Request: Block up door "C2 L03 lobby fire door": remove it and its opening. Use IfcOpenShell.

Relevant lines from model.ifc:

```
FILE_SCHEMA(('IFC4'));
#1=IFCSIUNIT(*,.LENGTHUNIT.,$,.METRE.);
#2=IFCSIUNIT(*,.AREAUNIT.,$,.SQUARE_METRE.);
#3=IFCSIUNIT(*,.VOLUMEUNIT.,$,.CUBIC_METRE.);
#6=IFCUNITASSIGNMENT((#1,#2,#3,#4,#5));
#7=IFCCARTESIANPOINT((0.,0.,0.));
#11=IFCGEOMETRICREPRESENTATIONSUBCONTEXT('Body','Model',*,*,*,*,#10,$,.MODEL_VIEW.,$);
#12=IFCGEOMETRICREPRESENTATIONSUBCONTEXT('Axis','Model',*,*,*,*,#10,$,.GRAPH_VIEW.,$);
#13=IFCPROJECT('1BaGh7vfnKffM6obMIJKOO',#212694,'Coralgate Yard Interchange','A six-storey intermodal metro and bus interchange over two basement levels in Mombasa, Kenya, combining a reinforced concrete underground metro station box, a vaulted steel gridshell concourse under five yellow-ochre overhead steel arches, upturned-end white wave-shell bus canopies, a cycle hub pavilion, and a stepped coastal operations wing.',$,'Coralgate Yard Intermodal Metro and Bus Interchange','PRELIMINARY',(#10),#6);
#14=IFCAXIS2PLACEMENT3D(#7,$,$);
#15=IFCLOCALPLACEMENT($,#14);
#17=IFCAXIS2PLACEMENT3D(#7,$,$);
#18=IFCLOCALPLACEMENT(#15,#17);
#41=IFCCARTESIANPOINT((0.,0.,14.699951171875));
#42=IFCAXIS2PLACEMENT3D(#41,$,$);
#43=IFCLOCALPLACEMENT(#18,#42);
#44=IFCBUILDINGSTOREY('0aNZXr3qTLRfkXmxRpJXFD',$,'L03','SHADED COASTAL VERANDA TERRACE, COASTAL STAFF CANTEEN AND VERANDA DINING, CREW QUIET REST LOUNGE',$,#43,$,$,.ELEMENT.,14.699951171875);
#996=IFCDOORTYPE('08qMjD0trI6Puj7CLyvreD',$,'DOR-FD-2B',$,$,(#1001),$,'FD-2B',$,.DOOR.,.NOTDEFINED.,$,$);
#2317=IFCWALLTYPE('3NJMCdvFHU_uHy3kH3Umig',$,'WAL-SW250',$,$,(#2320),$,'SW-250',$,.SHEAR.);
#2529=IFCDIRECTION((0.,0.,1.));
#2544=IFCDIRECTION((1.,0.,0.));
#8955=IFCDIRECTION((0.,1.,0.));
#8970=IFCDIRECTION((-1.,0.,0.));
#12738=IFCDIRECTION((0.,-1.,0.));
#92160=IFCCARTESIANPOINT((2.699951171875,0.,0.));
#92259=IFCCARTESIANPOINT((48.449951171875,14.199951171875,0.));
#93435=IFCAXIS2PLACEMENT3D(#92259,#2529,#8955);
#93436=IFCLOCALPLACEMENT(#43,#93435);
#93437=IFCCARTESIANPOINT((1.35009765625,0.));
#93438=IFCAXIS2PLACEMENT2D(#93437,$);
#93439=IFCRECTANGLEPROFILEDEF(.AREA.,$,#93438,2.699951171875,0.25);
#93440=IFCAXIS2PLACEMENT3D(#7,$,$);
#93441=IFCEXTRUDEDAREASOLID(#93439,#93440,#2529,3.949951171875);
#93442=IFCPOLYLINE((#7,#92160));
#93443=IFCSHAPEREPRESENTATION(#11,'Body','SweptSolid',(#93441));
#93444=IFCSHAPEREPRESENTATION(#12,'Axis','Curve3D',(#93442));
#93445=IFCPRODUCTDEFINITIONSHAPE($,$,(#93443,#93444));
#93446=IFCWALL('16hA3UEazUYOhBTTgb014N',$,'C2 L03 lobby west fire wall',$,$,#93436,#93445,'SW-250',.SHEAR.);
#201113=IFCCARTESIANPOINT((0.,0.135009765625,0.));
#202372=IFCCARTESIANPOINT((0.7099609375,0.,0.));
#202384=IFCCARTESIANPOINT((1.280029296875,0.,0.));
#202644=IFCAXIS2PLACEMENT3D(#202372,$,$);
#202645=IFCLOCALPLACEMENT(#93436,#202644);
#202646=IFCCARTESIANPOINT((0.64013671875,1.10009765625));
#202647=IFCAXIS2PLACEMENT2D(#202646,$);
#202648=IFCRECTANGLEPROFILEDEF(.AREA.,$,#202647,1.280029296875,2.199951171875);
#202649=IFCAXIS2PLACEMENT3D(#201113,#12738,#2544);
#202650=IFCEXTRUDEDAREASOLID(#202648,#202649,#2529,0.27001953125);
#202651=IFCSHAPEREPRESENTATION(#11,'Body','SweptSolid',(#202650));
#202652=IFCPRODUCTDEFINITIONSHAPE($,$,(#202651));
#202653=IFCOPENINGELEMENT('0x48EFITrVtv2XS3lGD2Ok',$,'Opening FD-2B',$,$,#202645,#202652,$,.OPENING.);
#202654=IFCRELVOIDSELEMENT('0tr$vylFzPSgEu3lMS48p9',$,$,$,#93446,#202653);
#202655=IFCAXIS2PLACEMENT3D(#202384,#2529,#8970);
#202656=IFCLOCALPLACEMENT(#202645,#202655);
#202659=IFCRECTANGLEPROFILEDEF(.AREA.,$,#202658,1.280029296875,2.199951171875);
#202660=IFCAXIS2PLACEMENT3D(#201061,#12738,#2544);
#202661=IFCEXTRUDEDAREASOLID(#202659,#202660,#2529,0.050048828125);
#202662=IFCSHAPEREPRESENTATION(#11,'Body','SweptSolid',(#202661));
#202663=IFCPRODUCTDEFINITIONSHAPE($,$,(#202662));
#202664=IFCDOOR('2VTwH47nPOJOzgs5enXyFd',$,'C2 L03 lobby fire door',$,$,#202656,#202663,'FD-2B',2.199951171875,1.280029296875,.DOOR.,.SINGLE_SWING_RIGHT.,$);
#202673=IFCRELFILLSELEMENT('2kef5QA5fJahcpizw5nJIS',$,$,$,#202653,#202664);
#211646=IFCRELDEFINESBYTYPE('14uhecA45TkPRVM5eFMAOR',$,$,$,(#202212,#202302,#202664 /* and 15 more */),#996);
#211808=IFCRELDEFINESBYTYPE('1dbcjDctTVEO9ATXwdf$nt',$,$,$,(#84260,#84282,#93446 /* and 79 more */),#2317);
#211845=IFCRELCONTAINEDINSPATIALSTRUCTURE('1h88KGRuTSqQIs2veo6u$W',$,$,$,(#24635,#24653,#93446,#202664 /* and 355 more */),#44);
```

```python
import ifcopenshell
import ifcopenshell.api.feature
import ifcopenshell.api.root
import ifcopenshell.geom
import ifcopenshell.util.shape

model = ifcopenshell.open("model.ifc")
settings = ifcopenshell.geom.settings()


def volume(element):
    """Net volume in cubic metres, openings subtracted."""
    shape = ifcopenshell.geom.create_shape(settings, element)
    return ifcopenshell.util.shape.get_volume(shape.geometry)


door = model.by_id(202664)
opening = door.FillsVoids[0].RelatingOpeningElement
wall = opening.VoidsElements[0].RelatingBuildingElement
before = volume(wall)

ifcopenshell.api.root.remove_product(model, product=door)
ifcopenshell.api.feature.remove_feature(model, feature=opening)

after = volume(wall)

print(f"wall volume {before:.3f} -> {after:.3f} m3")

model.write("model_edited.ifc")
```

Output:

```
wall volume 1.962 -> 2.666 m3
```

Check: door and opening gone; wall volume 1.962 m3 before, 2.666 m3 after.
